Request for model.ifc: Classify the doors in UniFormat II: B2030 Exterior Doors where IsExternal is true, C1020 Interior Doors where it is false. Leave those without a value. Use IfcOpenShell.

First a look at what the model holds.

```python
import ifcopenshell
import ifcopenshell.util.element

model = ifcopenshell.open("model.ifc")
print(model.schema)
print("classifications:", [c.Name for c in model.by_type("IfcClassification")])
values = [ifcopenshell.util.element.get_pset(e, "Pset_DoorCommon", "IsExternal") for e in model.by_type("IfcDoor")]
for value in (True, False, None):
    print("IsExternal", value, values.count(value))
```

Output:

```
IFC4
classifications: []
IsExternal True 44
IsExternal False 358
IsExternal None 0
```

```python
import ifcopenshell
import ifcopenshell.api.classification
import ifcopenshell.util.element

model = ifcopenshell.open("model.ifc")

system = ifcopenshell.api.classification.add_classification(model, classification="UniFormat II")

doors = model.by_type("IfcDoor")
external = {e: ifcopenshell.util.element.get_pset(e, "Pset_DoorCommon", "IsExternal") for e in doors}
for flag, code, name in ((True, "B2030", "Exterior Doors"), (False, "C1020", "Interior Doors")):
    products = [e for e in doors if external[e] is flag]
    ifcopenshell.api.classification.add_reference(
        model, products=products, classification=system, identification=code, name=name
    )
    print(code, len(products))

model.write("model_v2.ifc")
```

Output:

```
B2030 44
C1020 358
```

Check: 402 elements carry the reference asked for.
